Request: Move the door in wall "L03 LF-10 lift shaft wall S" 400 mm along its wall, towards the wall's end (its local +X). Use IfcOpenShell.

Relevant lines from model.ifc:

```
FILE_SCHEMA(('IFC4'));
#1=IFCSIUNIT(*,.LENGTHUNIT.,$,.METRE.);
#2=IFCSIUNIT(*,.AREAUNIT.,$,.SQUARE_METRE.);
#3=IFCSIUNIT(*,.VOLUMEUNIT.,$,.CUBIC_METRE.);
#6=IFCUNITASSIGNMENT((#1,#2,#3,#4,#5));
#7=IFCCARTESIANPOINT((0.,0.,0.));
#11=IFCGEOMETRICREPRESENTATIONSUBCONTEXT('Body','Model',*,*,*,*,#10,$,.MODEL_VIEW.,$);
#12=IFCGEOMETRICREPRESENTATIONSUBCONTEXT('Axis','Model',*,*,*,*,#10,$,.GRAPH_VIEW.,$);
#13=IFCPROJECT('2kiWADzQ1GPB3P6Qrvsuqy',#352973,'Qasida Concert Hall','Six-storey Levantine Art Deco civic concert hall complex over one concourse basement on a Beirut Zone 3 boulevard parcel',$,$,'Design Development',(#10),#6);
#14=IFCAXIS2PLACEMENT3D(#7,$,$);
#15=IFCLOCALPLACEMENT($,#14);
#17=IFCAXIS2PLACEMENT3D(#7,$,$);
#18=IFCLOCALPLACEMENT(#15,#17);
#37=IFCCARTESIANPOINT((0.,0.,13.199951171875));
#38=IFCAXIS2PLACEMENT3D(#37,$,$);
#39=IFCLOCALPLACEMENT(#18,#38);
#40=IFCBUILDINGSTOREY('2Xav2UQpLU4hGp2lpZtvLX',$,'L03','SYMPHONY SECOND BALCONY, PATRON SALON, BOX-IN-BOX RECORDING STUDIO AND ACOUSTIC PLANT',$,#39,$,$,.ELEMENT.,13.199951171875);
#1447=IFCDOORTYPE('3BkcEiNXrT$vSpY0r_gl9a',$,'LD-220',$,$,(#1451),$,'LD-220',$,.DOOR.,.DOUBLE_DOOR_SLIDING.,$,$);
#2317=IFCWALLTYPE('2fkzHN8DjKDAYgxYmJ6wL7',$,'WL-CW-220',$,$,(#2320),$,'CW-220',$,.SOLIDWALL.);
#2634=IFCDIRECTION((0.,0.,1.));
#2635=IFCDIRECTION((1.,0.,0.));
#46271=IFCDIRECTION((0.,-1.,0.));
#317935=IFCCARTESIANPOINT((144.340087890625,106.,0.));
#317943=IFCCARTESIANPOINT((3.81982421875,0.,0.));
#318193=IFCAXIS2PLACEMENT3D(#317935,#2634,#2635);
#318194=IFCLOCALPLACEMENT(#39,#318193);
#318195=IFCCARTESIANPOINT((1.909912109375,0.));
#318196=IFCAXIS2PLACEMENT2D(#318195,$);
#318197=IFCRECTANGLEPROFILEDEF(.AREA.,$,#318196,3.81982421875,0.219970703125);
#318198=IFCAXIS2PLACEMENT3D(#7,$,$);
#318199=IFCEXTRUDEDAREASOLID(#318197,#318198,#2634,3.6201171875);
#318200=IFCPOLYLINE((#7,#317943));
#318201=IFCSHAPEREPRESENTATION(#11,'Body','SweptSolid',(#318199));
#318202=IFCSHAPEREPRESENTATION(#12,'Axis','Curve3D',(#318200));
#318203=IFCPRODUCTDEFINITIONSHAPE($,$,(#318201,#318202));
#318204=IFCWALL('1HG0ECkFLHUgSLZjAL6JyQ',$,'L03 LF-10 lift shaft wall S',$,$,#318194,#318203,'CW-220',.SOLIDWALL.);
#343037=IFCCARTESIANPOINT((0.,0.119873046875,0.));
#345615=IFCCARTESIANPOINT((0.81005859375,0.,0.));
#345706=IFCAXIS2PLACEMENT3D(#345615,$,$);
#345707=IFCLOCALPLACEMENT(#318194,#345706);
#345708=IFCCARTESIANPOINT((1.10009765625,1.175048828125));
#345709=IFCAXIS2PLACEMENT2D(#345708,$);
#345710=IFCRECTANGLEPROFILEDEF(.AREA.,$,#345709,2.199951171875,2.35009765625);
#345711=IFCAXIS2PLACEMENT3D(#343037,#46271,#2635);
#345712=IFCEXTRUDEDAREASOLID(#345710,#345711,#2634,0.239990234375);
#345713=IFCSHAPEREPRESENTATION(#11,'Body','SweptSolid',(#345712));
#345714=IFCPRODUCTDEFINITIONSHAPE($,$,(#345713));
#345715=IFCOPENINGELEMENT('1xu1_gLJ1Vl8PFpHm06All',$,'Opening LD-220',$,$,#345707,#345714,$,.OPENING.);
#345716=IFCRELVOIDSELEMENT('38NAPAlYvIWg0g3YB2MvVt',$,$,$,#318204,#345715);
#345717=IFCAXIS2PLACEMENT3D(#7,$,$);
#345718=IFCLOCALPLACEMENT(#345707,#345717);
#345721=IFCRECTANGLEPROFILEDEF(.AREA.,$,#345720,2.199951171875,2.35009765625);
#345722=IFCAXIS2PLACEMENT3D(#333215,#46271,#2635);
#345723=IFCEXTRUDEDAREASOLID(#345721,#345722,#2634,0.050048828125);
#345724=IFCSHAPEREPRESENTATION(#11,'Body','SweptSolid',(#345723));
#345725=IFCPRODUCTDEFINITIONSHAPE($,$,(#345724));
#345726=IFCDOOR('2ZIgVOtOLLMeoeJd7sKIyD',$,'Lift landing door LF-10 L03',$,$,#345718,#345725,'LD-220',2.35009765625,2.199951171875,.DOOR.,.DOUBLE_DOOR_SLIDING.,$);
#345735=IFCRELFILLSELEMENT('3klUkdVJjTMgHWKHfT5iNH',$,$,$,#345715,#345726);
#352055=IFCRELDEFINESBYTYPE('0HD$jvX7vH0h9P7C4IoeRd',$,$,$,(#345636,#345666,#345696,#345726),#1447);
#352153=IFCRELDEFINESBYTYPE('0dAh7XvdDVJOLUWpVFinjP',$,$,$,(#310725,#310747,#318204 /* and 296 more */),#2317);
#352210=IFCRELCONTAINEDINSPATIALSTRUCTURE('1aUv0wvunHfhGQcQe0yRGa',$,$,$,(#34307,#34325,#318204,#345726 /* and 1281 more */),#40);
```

```python
import ifcopenshell
import ifcopenshell.api.geometry
import ifcopenshell.util.placement
import ifcopenshell.util.unit

model = ifcopenshell.open("model.ifc")
unit_scale = ifcopenshell.util.unit.calculate_unit_scale(model)

door = model.by_guid("2ZIgVOtOLLMeoeJd7sKIyD")
opening = door.FillsVoids[0].RelatingOpeningElement
wall = opening.VoidsElements[0].RelatingBuildingElement

wall_matrix = ifcopenshell.util.placement.get_local_placement(wall.ObjectPlacement)
shift = wall_matrix[:3, 0] * 0.4 / unit_scale
before = ifcopenshell.util.placement.get_local_placement(door.ObjectPlacement)[:3, 3].copy()

# The door is placed relative to its opening, so it follows when the opening moves.
matrix = ifcopenshell.util.placement.get_local_placement(opening.ObjectPlacement)
matrix[:3, 3] += shift
ifcopenshell.api.geometry.edit_object_placement(
    model, product=opening, matrix=matrix, is_si=False, should_transform_children=True
)

after = ifcopenshell.util.placement.get_local_placement(door.ObjectPlacement)[:3, 3]
print("door moved by", (after - before).round(3) + 0.0)

model.write("model_edited.ifc")
```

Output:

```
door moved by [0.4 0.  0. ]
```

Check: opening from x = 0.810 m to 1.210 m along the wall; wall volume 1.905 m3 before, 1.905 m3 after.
